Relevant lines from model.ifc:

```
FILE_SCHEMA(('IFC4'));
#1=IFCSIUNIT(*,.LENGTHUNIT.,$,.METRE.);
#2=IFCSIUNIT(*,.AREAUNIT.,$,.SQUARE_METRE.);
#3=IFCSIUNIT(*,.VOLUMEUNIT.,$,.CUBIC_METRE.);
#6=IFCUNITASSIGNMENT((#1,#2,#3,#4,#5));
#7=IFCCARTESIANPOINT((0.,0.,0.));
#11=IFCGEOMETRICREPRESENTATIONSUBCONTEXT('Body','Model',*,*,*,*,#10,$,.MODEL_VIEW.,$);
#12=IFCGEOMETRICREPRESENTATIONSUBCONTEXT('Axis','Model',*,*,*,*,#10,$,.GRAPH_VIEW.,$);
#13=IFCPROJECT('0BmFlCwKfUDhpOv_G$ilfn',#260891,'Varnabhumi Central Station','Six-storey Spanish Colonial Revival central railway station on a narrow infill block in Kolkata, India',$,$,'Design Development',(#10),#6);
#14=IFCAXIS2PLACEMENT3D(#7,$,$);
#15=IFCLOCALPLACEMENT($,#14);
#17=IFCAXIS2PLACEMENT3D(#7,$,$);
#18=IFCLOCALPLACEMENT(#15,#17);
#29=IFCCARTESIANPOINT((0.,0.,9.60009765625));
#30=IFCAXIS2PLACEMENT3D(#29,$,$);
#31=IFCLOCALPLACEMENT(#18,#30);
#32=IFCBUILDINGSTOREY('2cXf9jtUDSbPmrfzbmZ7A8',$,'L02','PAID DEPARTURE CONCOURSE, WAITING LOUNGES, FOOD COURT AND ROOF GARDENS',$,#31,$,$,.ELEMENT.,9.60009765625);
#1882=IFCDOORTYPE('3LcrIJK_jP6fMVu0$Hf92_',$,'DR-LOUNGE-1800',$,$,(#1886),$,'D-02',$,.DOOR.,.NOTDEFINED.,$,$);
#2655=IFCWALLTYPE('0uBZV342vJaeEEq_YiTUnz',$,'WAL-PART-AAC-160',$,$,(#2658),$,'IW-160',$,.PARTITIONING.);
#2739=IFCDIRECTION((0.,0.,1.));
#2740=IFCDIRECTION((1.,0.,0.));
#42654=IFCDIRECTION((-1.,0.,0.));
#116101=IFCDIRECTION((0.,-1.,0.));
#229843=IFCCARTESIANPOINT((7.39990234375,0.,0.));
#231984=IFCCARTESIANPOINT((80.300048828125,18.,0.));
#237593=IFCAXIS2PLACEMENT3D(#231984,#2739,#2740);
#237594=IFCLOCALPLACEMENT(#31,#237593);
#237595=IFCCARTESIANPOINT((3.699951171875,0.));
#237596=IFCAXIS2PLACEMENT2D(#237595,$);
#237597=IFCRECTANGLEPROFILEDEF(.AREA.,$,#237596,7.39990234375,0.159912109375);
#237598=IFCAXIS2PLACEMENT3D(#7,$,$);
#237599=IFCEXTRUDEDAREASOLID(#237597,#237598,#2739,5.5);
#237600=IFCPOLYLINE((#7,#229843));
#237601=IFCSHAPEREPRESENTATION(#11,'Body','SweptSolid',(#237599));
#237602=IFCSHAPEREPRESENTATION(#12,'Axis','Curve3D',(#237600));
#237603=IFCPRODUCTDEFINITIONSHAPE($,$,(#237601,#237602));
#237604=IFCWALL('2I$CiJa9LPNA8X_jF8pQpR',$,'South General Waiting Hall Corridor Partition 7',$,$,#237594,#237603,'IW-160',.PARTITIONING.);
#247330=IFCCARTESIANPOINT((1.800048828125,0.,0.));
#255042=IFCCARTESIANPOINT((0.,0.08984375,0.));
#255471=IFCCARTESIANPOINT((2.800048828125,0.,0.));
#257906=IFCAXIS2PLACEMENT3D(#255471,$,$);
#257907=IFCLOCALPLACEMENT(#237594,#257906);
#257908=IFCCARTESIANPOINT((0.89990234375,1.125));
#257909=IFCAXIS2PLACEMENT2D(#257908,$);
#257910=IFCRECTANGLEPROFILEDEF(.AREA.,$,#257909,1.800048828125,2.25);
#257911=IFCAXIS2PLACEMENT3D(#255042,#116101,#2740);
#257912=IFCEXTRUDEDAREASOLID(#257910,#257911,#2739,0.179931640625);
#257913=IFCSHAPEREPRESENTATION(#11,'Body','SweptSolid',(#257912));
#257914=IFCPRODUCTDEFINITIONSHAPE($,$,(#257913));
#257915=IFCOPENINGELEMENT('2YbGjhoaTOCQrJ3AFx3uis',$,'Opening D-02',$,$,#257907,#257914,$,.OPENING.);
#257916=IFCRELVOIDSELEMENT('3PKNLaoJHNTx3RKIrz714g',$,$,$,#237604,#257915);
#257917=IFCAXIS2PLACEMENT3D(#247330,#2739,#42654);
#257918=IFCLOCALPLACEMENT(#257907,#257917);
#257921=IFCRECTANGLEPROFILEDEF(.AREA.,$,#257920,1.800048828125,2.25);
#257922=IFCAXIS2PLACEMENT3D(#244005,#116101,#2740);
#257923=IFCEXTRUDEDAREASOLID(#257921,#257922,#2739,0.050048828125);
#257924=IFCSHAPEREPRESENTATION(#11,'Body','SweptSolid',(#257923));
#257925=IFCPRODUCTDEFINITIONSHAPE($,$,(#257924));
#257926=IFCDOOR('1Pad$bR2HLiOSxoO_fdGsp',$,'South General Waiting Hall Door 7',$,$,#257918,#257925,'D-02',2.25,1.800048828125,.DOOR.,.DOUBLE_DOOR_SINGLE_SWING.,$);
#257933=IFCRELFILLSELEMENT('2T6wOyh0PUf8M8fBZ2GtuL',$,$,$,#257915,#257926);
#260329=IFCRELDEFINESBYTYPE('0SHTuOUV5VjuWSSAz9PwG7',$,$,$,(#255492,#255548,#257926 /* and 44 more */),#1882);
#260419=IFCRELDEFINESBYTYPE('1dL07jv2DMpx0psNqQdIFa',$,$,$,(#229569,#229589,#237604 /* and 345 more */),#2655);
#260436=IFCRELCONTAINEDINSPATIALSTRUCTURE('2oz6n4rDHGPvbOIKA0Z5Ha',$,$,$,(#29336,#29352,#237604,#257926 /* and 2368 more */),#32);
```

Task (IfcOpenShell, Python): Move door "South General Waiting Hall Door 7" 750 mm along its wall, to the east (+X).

```python
import ifcopenshell
import ifcopenshell.api.geometry
import ifcopenshell.util.placement

model = ifcopenshell.open("model.ifc")

door = model.by_id(257926)
opening = door.FillsVoids[0].RelatingOpeningElement
wall = opening.VoidsElements[0].RelatingBuildingElement

wall_matrix = ifcopenshell.util.placement.get_local_placement(wall.ObjectPlacement)
shift = wall_matrix[:3, 0] * 0.75
before = ifcopenshell.util.placement.get_local_placement(door.ObjectPlacement)[:3, 3].copy()

# The door is placed relative to its opening, so it follows when the opening moves.
matrix = ifcopenshell.util.placement.get_local_placement(opening.ObjectPlacement)
matrix[:3, 3] += shift
ifcopenshell.api.geometry.edit_object_placement(
    model, product=opening, matrix=matrix, is_si=False, should_transform_children=True
)

after = ifcopenshell.util.placement.get_local_placement(door.ObjectPlacement)[:3, 3]
print("door moved by", (after - before).round(3) + 0.0)

model.write("model-out.ifc")
```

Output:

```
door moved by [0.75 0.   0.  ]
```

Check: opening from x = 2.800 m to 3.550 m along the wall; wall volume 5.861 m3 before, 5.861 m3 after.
